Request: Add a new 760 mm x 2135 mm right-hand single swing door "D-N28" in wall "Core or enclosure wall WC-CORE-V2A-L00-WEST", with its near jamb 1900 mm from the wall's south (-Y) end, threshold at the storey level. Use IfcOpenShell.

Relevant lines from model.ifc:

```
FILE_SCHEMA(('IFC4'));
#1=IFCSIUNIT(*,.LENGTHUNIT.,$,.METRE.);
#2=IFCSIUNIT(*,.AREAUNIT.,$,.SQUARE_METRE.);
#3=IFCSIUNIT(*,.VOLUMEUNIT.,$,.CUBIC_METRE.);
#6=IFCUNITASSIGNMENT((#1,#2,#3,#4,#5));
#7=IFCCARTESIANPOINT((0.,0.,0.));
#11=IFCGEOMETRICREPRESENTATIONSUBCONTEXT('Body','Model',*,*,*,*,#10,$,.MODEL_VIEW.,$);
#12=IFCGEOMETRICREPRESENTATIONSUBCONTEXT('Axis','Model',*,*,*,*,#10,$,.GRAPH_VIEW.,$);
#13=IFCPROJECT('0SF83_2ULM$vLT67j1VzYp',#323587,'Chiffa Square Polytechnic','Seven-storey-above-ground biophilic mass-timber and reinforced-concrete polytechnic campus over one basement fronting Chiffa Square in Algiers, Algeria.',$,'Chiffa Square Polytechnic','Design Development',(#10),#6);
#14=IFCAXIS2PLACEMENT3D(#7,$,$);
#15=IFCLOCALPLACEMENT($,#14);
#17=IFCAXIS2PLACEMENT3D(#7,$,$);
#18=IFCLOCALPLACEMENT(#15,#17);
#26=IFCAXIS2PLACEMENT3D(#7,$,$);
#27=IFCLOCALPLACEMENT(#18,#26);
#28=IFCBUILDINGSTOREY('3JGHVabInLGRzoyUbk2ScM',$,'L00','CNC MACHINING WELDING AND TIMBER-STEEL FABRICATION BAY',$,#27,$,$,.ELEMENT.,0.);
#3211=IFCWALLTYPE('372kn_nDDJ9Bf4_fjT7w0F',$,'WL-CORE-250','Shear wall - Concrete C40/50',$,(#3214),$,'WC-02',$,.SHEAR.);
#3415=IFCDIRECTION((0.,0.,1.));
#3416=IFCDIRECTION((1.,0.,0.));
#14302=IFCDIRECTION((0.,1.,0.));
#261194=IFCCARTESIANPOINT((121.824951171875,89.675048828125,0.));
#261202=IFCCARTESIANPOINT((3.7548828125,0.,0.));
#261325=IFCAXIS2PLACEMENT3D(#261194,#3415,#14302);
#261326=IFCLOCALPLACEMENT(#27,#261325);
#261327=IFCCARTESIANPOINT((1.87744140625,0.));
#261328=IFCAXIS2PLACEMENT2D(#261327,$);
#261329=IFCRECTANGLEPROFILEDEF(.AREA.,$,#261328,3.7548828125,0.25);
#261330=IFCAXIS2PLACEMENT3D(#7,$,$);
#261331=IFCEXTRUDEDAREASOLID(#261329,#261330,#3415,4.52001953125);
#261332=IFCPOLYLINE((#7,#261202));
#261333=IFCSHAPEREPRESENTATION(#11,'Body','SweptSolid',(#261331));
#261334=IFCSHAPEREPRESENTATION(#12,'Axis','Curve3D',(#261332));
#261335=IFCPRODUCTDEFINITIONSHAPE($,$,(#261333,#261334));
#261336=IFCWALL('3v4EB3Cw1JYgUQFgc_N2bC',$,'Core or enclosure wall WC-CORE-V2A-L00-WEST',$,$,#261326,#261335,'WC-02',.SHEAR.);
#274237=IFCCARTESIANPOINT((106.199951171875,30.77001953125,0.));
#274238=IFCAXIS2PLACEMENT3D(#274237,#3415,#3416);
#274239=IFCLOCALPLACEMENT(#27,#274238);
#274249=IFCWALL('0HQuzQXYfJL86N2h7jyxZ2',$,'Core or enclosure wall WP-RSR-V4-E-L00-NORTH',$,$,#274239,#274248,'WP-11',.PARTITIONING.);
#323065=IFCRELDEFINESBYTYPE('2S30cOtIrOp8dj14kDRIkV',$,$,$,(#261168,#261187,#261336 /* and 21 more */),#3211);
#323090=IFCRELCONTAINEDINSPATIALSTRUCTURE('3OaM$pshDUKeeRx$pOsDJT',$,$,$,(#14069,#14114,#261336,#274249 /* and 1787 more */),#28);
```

```python
import numpy as np
import ifcopenshell
import ifcopenshell.api.feature
import ifcopenshell.api.geometry
import ifcopenshell.api.root
import ifcopenshell.api.spatial
import ifcopenshell.geom
import ifcopenshell.util.element
import ifcopenshell.util.placement
import ifcopenshell.util.representation
import ifcopenshell.util.shape
import ifcopenshell.util.unit

model = ifcopenshell.open("model.ifc")
unit_scale = ifcopenshell.util.unit.calculate_unit_scale(model)
settings = ifcopenshell.geom.settings()


def volume(element):
    """Net volume in cubic metres, openings subtracted."""
    shape = ifcopenshell.geom.create_shape(settings, element)
    return ifcopenshell.util.shape.get_volume(shape.geometry)


wall = model.by_guid("3v4EB3Cw1JYgUQFgc_N2bC")
storey = ifcopenshell.util.element.get_container(wall, ifc_class="IfcBuildingStorey")
context = ifcopenshell.util.representation.get_context(model, "Model", "Body", "MODEL_VIEW")
before = volume(wall)

width, height, from_end, sill = 0.76, 2.135, 1.9, 0.0  # metres

# The wall runs along its own X axis, and the end named is its -X end.
wall_shape = ifcopenshell.geom.create_shape(settings, wall)
x, y, z = ifcopenshell.util.shape.get_vertices(wall_shape.geometry).T
start = x.min() + from_end
face, thickness = float(y.min()), float(y.max() - y.min())
wall_matrix = ifcopenshell.util.placement.get_local_placement(wall.ObjectPlacement)
level = ifcopenshell.util.placement.get_local_placement(storey.ObjectPlacement)[2, 3]


def in_wall(x, y):
    """Placement at x, y metres in the wall's axes, at sill height."""
    matrix = wall_matrix.copy()
    matrix[:, 3] = wall_matrix @ np.array([x / unit_scale, y / unit_scale, 0.0, 1.0])
    matrix[2, 3] = level + sill / unit_scale
    return matrix


# Opening: a box that overshoots both wall faces by 50 mm.
opening = ifcopenshell.api.root.create_entity(model, ifc_class="IfcOpeningElement", predefined_type="OPENING")
box = ifcopenshell.api.geometry.add_wall_representation(
    model, context=context, length=width, height=height, thickness=thickness + 0.1
)
ifcopenshell.api.geometry.assign_representation(model, product=opening, representation=box)
ifcopenshell.api.geometry.edit_object_placement(model, product=opening, matrix=in_wall(start, face - 0.05), is_si=False)
ifcopenshell.api.feature.add_feature(model, feature=opening, element=wall)

door = ifcopenshell.api.root.create_entity(model, ifc_class="IfcDoor", name="D-N28", predefined_type="DOOR")
door.OverallWidth, door.OverallHeight = width / unit_scale, height / unit_scale
door.OperationType = "SINGLE_SWING_RIGHT"
body = ifcopenshell.api.geometry.add_door_representation(
    model,
    context=context,
    overall_width=door.OverallWidth,
    overall_height=door.OverallHeight,
    operation_type="SINGLE_SWING_RIGHT",
    lining_properties={"LiningDepth": thickness / unit_scale, "ThresholdDepth": thickness / unit_scale},
)
ifcopenshell.api.geometry.assign_representation(model, product=door, representation=body)
ifcopenshell.api.spatial.assign_container(model, products=[door], relating_structure=storey)
ifcopenshell.api.feature.add_filling(model, opening=opening, element=door)

# The lining spans the wall, so the door starts at the wall face.
ifcopenshell.api.geometry.edit_object_placement(model, product=door, matrix=in_wall(start, face), is_si=False)

after = volume(wall)

print(f"wall volume {before:.3f} -> {after:.3f} m3")

model.write("model-out.ifc")
```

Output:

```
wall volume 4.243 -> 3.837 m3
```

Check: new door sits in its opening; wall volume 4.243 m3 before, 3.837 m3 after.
